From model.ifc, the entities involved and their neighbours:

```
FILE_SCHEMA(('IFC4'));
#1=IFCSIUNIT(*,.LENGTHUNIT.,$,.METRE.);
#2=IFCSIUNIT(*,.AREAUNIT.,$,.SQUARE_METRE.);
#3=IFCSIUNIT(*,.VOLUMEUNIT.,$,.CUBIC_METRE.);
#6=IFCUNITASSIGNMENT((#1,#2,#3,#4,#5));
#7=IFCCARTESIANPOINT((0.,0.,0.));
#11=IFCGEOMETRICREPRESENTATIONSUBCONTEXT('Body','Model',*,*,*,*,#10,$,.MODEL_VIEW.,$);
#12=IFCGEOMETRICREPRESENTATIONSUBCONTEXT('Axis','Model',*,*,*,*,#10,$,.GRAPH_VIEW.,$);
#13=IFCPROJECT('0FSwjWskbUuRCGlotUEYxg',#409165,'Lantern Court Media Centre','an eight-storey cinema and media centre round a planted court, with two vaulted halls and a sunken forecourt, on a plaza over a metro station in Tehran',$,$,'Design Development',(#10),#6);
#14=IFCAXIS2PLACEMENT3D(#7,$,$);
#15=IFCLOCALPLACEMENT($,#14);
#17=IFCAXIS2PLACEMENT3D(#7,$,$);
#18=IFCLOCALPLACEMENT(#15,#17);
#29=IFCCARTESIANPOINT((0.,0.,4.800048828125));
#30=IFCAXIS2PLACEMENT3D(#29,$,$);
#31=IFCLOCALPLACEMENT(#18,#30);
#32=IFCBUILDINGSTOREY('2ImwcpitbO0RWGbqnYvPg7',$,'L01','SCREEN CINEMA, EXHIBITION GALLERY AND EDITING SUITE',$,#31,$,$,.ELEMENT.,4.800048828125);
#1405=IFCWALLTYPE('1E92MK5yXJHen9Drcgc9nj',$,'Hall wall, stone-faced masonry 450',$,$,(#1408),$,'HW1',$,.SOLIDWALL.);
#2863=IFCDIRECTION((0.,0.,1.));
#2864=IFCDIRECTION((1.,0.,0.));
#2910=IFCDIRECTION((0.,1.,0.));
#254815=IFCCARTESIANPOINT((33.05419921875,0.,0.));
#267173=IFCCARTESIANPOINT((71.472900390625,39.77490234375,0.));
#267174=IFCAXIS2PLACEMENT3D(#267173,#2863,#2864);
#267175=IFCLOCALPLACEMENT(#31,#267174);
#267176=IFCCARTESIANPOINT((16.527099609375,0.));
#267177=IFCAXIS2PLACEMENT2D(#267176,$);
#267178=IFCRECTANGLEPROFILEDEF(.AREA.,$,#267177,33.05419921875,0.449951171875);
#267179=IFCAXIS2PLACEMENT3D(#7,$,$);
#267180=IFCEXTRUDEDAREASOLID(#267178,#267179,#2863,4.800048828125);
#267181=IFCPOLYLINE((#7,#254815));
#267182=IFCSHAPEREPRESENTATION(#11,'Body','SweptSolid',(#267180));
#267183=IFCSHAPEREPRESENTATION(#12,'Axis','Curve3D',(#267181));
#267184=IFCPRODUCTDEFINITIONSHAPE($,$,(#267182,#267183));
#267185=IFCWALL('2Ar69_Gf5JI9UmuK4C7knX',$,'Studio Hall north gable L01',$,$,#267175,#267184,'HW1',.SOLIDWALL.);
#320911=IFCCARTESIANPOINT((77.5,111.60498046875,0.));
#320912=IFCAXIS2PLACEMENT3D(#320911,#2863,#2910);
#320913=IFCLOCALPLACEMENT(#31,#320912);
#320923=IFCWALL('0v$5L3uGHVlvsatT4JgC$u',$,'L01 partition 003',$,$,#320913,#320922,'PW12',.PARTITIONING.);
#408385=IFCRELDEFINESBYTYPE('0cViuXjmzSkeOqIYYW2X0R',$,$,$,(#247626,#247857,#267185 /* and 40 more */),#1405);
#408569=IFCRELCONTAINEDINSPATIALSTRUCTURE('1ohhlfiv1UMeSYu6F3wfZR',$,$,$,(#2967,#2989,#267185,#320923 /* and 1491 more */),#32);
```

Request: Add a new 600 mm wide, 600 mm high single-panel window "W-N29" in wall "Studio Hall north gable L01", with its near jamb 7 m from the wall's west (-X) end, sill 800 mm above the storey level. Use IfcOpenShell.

```python
import numpy as np
import ifcopenshell
import ifcopenshell.api.feature
import ifcopenshell.api.geometry
import ifcopenshell.api.root
import ifcopenshell.api.spatial
import ifcopenshell.geom
import ifcopenshell.util.element
import ifcopenshell.util.placement
import ifcopenshell.util.representation
import ifcopenshell.util.shape
import ifcopenshell.util.unit

model = ifcopenshell.open("model.ifc")
unit_scale = ifcopenshell.util.unit.calculate_unit_scale(model)
settings = ifcopenshell.geom.settings()


def volume(element):
    """Net volume in cubic metres, openings subtracted."""
    shape = ifcopenshell.geom.create_shape(settings, element)
    return ifcopenshell.util.shape.get_volume(shape.geometry)


wall = model.by_guid("2Ar69_Gf5JI9UmuK4C7knX")
storey = ifcopenshell.util.element.get_container(wall, ifc_class="IfcBuildingStorey")
context = ifcopenshell.util.representation.get_context(model, "Model", "Body", "MODEL_VIEW")
before = volume(wall)

width, height, from_end, sill = 0.6, 0.6, 7, 0.8  # metres

# The wall runs along its own X axis, and the end named is its -X end.
wall_shape = ifcopenshell.geom.create_shape(settings, wall)
x, y, z = ifcopenshell.util.shape.get_vertices(wall_shape.geometry).T
start = x.min() + from_end
face, thickness = float(y.min()), float(y.max() - y.min())
wall_matrix = ifcopenshell.util.placement.get_local_placement(wall.ObjectPlacement)
level = ifcopenshell.util.placement.get_local_placement(storey.ObjectPlacement)[2, 3]


def in_wall(x, y):
    """Placement at x, y metres in the wall's axes, at sill height."""
    matrix = wall_matrix.copy()
    matrix[:, 3] = wall_matrix @ np.array([x / unit_scale, y / unit_scale, 0.0, 1.0])
    matrix[2, 3] = level + sill / unit_scale
    return matrix


# Opening: a box that overshoots both wall faces by 50 mm.
opening = ifcopenshell.api.root.create_entity(model, ifc_class="IfcOpeningElement", predefined_type="OPENING")
box = ifcopenshell.api.geometry.add_wall_representation(
    model, context=context, length=width, height=height, thickness=thickness + 0.1
)
ifcopenshell.api.geometry.assign_representation(model, product=opening, representation=box)
ifcopenshell.api.geometry.edit_object_placement(model, product=opening, matrix=in_wall(start, face - 0.05), is_si=False)
ifcopenshell.api.feature.add_feature(model, feature=opening, element=wall)

window = ifcopenshell.api.root.create_entity(model, ifc_class="IfcWindow", name="W-N29", predefined_type="WINDOW")
window.OverallWidth, window.OverallHeight = width / unit_scale, height / unit_scale
window.PartitioningType = "SINGLE_PANEL"
body = ifcopenshell.api.geometry.add_window_representation(
    model,
    context=context,
    overall_width=window.OverallWidth,
    overall_height=window.OverallHeight,
    partition_type="SINGLE_PANEL",
)
ifcopenshell.api.geometry.assign_representation(model, product=window, representation=body)
ifcopenshell.api.spatial.assign_container(model, products=[window], relating_structure=storey)
ifcopenshell.api.feature.add_filling(model, opening=opening, element=window)

# Centre the window in the wall's thickness.
ifcopenshell.api.geometry.edit_object_placement(model, product=window, matrix=in_wall(start, face), is_si=False)
window_shape = ifcopenshell.geom.create_shape(settings, window)
depth = ifcopenshell.util.shape.get_vertices(window_shape.geometry)[:, 1]
offset = face + thickness / 2 - (depth.min() + depth.max()) / 2
ifcopenshell.api.geometry.edit_object_placement(model, product=window, matrix=in_wall(start, offset), is_si=False)

after = volume(wall)

print(f"wall volume {before:.3f} -> {after:.3f} m3")

model.write("model_edited.ifc")
```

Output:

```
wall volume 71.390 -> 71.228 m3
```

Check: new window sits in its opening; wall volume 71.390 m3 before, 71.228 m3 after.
